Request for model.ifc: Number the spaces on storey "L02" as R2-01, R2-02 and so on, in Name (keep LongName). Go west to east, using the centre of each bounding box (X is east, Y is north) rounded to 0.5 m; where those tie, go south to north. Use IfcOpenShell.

First a look at what the model holds.

```python
import ifcopenshell
import ifcopenshell.util.element
import ifcopenshell.util.placement

model = ifcopenshell.open("model.ifc")
print(model.schema)
storey = next(s for s in model.by_type("IfcBuildingStorey") if s.Name == "L02")
spaces = [e for e in ifcopenshell.util.element.get_decomposition(storey) if e.is_a("IfcSpace")]
for e in sorted(spaces, key=lambda e: e.id()):
    origin = ifcopenshell.util.placement.get_local_placement(e.ObjectPlacement)[:3, 3]
    print(e.id(), e.Name, e.LongName, origin.round(2) + 0.0, sep=" | ")
```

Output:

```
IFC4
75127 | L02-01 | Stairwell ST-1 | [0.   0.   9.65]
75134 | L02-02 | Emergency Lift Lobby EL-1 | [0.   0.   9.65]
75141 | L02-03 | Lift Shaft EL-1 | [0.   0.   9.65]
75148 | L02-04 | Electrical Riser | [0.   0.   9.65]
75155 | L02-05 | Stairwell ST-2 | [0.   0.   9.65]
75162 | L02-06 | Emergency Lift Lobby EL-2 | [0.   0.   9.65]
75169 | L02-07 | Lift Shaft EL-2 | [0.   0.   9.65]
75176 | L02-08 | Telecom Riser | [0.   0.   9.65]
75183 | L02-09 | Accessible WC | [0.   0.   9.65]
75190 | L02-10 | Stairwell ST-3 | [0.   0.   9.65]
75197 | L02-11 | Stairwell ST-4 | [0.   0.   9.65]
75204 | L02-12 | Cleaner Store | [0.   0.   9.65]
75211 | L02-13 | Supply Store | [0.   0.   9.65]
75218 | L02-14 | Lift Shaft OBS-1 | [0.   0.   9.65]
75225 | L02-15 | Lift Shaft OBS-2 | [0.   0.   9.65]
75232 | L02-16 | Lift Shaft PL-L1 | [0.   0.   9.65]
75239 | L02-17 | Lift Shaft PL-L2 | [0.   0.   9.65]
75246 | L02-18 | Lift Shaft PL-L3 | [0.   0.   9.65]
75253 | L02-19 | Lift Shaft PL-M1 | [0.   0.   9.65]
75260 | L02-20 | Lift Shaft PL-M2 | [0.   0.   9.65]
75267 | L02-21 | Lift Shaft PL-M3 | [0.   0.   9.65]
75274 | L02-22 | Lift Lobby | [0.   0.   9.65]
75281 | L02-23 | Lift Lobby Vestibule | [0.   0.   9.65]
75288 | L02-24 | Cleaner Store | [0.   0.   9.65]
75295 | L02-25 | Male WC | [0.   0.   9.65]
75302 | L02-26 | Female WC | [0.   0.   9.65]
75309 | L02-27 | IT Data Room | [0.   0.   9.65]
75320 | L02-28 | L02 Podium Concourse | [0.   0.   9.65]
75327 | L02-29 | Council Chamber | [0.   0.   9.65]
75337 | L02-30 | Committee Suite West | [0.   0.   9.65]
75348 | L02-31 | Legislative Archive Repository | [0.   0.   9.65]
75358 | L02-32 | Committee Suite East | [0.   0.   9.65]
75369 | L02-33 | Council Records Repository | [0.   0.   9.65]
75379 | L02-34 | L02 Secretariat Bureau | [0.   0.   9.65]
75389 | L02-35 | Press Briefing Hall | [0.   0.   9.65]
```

```python
import ifcopenshell
import ifcopenshell.geom
import ifcopenshell.util.element
import ifcopenshell.util.shape

model = ifcopenshell.open("model.ifc")
settings = ifcopenshell.geom.settings()
settings.set("use-world-coords", True)


def centre(element):
    shape = ifcopenshell.geom.create_shape(settings, element)
    return ifcopenshell.util.shape.get_bbox_centroid(shape.geometry)


storey = next(s for s in model.by_type("IfcBuildingStorey") if s.Name == "L02")
spaces = [e for e in ifcopenshell.util.element.get_decomposition(storey) if e.is_a("IfcSpace")]

# Insertion points can sit at a corner or the storey origin, so sort by the geometry (in metres).
centres = {e: centre(e) for e in spaces}
spaces.sort(key=lambda e: (round(centres[e][0] / 0.5), centres[e][1]))

for i, e in enumerate(spaces, start=1):
    number = f"R2-{i:02d}"
    e.Name = number
    print(e.id(), number)

model.write("model_rev.ifc")
```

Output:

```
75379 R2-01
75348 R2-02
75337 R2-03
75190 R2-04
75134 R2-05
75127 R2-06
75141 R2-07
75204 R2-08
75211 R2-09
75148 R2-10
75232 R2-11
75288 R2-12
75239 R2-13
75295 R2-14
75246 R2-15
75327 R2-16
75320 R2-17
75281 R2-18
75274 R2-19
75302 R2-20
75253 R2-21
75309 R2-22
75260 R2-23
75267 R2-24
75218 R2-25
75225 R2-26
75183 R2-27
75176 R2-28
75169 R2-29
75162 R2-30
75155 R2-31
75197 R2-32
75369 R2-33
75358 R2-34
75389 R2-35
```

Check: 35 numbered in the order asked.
